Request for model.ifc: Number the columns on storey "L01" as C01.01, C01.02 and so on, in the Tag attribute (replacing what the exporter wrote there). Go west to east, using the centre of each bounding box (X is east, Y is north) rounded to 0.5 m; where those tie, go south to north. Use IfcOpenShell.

First a look at what the model holds.

```python
import ifcopenshell
import ifcopenshell.util.element
import ifcopenshell.util.placement

model = ifcopenshell.open("model.ifc")
print(model.schema)
storey = next(s for s in model.by_type("IfcBuildingStorey") if s.Name == "L01")
columns = [e for e in ifcopenshell.util.element.get_decomposition(storey) if e.is_a("IfcColumn")]
for e in sorted(columns, key=lambda e: e.id()):
    origin = ifcopenshell.util.placement.get_local_placement(e.ObjectPlacement)[:3, 3]
    print(e.id(), e.Tag, e.Name, origin.round(2) + 0.0, sep=" | ")
```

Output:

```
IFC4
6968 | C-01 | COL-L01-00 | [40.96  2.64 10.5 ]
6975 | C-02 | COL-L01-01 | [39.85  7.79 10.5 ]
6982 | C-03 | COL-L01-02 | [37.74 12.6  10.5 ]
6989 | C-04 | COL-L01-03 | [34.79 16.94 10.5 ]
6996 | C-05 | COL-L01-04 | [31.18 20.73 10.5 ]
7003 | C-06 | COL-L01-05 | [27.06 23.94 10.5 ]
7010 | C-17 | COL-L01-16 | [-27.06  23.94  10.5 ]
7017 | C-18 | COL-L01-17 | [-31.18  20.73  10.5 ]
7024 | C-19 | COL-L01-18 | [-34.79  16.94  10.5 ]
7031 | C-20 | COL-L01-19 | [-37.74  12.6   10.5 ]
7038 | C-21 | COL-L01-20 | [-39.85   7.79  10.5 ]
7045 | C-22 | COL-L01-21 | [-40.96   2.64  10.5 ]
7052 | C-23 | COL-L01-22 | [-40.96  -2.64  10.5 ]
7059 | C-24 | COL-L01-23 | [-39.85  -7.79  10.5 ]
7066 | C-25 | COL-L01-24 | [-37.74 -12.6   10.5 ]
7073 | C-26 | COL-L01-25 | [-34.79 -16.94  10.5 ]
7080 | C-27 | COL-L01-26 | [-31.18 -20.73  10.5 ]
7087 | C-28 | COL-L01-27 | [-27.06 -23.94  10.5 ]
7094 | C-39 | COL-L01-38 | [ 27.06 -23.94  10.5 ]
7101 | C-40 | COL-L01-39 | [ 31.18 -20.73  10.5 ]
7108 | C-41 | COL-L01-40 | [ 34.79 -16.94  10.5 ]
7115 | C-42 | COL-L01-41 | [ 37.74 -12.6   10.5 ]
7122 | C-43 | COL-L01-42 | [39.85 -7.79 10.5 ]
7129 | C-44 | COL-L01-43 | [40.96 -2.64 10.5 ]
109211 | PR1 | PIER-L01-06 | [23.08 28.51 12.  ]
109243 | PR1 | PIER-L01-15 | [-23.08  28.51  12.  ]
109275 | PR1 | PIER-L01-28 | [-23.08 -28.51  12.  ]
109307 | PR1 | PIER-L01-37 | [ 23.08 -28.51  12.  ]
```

```python
import ifcopenshell
import ifcopenshell.geom
import ifcopenshell.util.element
import ifcopenshell.util.shape

model = ifcopenshell.open("model.ifc")
settings = ifcopenshell.geom.settings()
settings.set("use-world-coords", True)


def centre(element):
    shape = ifcopenshell.geom.create_shape(settings, element)
    return ifcopenshell.util.shape.get_bbox_centroid(shape.geometry)


storey = next(s for s in model.by_type("IfcBuildingStorey") if s.Name == "L01")
columns = [e for e in ifcopenshell.util.element.get_decomposition(storey) if e.is_a("IfcColumn")]

# Insertion points can sit at a corner or the storey origin, so sort by the geometry (in metres).
centres = {e: centre(e) for e in columns}
columns.sort(key=lambda e: (round(centres[e][0] / 0.5), centres[e][1]))

for i, e in enumerate(columns, start=1):
    number = f"C01.{i:02d}"
    e.Tag = number
    print(e.id(), number)

model.write("model_edited.ifc")
```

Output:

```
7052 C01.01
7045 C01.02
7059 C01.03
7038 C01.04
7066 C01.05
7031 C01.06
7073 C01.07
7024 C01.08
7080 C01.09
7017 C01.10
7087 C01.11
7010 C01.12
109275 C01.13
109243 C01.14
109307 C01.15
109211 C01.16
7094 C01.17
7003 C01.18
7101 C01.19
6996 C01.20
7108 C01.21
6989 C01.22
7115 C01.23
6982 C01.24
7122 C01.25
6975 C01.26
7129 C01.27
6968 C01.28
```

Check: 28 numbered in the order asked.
